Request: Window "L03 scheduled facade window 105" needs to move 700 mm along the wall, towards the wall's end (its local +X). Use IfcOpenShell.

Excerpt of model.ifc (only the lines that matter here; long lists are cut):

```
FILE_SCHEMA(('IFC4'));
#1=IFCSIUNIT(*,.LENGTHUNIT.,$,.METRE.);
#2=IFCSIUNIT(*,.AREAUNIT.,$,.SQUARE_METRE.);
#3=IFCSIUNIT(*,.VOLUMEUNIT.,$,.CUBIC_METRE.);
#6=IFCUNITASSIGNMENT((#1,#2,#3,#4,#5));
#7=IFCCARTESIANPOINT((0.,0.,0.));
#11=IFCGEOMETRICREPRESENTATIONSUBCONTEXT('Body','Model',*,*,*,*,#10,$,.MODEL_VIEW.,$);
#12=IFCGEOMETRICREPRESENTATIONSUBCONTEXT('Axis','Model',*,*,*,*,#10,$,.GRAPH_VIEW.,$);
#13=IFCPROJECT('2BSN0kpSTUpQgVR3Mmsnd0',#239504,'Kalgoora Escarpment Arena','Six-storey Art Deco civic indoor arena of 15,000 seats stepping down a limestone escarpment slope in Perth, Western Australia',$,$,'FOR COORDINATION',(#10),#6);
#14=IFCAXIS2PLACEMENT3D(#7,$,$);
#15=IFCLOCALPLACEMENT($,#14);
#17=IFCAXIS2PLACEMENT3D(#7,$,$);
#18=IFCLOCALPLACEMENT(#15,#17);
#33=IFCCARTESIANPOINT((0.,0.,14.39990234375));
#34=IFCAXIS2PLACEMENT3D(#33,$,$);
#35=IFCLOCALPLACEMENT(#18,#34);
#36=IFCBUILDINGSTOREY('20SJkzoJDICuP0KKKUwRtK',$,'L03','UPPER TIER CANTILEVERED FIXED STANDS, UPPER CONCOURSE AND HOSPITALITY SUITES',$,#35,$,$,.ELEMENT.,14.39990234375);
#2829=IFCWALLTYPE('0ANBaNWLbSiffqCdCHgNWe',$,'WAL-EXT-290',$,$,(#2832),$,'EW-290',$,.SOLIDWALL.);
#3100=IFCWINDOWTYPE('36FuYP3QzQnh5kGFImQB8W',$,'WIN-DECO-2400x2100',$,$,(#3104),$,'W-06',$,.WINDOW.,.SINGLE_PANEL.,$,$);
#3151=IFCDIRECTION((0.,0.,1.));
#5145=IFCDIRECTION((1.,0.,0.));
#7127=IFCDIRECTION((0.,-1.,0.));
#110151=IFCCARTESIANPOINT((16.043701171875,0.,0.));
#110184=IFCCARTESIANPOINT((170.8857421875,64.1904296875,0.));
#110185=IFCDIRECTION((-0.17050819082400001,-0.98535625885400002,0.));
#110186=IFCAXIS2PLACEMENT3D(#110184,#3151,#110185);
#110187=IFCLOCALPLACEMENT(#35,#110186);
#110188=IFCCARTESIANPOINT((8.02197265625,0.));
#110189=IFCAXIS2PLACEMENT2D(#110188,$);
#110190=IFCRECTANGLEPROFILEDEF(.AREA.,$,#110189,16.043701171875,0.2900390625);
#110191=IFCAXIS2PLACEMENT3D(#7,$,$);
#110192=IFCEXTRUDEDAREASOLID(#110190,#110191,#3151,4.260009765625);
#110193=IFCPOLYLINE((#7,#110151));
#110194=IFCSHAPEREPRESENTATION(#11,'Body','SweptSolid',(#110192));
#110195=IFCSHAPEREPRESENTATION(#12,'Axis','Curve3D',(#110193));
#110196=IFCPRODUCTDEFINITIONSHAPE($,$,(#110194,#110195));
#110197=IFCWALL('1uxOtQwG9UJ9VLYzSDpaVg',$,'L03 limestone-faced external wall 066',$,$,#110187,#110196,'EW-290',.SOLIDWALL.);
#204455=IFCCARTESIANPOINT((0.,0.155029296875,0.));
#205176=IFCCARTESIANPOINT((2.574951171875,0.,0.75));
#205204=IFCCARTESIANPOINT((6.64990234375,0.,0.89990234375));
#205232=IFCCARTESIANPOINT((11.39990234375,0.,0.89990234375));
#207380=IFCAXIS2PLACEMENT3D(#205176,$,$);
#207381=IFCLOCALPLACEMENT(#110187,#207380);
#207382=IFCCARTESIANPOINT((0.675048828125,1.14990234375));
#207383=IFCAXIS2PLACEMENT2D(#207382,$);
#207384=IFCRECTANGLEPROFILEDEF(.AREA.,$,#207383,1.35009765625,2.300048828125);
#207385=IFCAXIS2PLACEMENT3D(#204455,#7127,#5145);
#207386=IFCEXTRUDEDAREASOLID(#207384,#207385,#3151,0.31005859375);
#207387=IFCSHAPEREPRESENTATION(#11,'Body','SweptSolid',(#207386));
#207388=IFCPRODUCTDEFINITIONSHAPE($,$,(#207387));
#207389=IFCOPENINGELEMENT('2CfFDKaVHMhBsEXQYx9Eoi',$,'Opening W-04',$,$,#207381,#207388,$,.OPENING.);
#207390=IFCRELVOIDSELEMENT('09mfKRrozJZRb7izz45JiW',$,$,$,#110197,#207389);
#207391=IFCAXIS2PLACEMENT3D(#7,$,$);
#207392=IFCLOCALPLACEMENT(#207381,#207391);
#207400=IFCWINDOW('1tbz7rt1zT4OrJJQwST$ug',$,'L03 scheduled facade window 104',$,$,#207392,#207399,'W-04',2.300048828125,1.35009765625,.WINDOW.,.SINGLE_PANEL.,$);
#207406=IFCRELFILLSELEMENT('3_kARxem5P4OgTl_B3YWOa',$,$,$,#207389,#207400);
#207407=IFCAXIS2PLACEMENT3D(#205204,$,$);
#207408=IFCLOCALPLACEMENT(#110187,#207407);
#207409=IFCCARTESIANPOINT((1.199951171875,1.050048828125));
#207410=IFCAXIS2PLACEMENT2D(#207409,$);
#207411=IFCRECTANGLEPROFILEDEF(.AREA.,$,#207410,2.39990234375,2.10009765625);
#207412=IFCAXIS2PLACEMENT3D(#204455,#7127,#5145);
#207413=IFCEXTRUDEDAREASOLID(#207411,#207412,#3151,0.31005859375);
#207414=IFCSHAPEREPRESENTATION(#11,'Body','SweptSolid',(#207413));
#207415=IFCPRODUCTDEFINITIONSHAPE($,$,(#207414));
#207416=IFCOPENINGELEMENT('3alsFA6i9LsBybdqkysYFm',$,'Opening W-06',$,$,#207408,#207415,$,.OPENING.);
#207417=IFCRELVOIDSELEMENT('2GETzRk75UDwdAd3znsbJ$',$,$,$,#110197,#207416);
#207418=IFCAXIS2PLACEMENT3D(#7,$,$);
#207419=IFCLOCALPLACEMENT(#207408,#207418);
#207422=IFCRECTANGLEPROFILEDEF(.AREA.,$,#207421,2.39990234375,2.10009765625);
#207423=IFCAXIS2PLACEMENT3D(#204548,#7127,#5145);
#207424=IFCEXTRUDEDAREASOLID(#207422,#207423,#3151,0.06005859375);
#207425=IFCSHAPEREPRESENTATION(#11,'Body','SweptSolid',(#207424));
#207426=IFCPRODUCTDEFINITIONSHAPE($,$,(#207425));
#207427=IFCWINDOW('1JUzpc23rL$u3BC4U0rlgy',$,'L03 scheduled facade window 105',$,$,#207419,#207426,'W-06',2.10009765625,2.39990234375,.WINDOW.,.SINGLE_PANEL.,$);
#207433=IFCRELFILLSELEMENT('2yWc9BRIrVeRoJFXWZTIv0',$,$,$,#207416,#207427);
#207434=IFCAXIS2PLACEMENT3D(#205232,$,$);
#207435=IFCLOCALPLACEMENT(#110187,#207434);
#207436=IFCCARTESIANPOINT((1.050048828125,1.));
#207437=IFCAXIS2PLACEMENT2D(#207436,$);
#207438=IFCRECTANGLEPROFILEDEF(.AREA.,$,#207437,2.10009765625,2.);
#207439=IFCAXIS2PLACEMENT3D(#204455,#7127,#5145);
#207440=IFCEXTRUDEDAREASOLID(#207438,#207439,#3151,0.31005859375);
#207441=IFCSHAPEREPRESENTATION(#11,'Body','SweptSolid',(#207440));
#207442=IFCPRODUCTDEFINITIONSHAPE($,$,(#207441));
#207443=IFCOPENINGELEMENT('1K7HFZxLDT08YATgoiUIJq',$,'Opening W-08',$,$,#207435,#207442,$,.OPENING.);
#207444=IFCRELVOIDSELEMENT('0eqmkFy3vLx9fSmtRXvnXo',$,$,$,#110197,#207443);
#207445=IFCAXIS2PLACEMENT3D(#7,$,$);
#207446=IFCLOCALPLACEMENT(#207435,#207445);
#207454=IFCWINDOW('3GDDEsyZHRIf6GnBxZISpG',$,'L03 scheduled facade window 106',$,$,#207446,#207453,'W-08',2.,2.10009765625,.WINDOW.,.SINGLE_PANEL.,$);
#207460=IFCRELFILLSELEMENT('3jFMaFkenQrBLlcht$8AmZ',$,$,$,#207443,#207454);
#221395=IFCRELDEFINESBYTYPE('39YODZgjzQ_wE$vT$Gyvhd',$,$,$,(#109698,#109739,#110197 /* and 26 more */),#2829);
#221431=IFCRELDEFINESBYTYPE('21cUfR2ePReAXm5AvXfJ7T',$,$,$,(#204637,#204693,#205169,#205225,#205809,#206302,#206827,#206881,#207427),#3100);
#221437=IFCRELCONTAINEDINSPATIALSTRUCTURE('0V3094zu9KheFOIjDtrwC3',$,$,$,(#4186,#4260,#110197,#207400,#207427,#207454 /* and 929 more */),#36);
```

```python
import ifcopenshell
import ifcopenshell.api.geometry
import ifcopenshell.util.placement
import ifcopenshell.util.unit

model = ifcopenshell.open("model.ifc")
unit_scale = ifcopenshell.util.unit.calculate_unit_scale(model)

window = model.by_guid("1JUzpc23rL$u3BC4U0rlgy")
opening = window.FillsVoids[0].RelatingOpeningElement
wall = opening.VoidsElements[0].RelatingBuildingElement

wall_matrix = ifcopenshell.util.placement.get_local_placement(wall.ObjectPlacement)
shift = wall_matrix[:3, 0] * 0.7 / unit_scale
before = ifcopenshell.util.placement.get_local_placement(window.ObjectPlacement)[:3, 3].copy()

# The window is placed relative to its opening, so it follows when the opening moves.
matrix = ifcopenshell.util.placement.get_local_placement(opening.ObjectPlacement)
matrix[:3, 3] += shift
ifcopenshell.api.geometry.edit_object_placement(
    model, product=opening, matrix=matrix, is_si=False, should_transform_children=True
)

after = ifcopenshell.util.placement.get_local_placement(window.ObjectPlacement)[:3, 3]
print("window moved by", (after - before).round(3) + 0.0)

model.write("model_rev.ifc")
```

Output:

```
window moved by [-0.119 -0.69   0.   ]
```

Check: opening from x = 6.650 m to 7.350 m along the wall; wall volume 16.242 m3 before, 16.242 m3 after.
